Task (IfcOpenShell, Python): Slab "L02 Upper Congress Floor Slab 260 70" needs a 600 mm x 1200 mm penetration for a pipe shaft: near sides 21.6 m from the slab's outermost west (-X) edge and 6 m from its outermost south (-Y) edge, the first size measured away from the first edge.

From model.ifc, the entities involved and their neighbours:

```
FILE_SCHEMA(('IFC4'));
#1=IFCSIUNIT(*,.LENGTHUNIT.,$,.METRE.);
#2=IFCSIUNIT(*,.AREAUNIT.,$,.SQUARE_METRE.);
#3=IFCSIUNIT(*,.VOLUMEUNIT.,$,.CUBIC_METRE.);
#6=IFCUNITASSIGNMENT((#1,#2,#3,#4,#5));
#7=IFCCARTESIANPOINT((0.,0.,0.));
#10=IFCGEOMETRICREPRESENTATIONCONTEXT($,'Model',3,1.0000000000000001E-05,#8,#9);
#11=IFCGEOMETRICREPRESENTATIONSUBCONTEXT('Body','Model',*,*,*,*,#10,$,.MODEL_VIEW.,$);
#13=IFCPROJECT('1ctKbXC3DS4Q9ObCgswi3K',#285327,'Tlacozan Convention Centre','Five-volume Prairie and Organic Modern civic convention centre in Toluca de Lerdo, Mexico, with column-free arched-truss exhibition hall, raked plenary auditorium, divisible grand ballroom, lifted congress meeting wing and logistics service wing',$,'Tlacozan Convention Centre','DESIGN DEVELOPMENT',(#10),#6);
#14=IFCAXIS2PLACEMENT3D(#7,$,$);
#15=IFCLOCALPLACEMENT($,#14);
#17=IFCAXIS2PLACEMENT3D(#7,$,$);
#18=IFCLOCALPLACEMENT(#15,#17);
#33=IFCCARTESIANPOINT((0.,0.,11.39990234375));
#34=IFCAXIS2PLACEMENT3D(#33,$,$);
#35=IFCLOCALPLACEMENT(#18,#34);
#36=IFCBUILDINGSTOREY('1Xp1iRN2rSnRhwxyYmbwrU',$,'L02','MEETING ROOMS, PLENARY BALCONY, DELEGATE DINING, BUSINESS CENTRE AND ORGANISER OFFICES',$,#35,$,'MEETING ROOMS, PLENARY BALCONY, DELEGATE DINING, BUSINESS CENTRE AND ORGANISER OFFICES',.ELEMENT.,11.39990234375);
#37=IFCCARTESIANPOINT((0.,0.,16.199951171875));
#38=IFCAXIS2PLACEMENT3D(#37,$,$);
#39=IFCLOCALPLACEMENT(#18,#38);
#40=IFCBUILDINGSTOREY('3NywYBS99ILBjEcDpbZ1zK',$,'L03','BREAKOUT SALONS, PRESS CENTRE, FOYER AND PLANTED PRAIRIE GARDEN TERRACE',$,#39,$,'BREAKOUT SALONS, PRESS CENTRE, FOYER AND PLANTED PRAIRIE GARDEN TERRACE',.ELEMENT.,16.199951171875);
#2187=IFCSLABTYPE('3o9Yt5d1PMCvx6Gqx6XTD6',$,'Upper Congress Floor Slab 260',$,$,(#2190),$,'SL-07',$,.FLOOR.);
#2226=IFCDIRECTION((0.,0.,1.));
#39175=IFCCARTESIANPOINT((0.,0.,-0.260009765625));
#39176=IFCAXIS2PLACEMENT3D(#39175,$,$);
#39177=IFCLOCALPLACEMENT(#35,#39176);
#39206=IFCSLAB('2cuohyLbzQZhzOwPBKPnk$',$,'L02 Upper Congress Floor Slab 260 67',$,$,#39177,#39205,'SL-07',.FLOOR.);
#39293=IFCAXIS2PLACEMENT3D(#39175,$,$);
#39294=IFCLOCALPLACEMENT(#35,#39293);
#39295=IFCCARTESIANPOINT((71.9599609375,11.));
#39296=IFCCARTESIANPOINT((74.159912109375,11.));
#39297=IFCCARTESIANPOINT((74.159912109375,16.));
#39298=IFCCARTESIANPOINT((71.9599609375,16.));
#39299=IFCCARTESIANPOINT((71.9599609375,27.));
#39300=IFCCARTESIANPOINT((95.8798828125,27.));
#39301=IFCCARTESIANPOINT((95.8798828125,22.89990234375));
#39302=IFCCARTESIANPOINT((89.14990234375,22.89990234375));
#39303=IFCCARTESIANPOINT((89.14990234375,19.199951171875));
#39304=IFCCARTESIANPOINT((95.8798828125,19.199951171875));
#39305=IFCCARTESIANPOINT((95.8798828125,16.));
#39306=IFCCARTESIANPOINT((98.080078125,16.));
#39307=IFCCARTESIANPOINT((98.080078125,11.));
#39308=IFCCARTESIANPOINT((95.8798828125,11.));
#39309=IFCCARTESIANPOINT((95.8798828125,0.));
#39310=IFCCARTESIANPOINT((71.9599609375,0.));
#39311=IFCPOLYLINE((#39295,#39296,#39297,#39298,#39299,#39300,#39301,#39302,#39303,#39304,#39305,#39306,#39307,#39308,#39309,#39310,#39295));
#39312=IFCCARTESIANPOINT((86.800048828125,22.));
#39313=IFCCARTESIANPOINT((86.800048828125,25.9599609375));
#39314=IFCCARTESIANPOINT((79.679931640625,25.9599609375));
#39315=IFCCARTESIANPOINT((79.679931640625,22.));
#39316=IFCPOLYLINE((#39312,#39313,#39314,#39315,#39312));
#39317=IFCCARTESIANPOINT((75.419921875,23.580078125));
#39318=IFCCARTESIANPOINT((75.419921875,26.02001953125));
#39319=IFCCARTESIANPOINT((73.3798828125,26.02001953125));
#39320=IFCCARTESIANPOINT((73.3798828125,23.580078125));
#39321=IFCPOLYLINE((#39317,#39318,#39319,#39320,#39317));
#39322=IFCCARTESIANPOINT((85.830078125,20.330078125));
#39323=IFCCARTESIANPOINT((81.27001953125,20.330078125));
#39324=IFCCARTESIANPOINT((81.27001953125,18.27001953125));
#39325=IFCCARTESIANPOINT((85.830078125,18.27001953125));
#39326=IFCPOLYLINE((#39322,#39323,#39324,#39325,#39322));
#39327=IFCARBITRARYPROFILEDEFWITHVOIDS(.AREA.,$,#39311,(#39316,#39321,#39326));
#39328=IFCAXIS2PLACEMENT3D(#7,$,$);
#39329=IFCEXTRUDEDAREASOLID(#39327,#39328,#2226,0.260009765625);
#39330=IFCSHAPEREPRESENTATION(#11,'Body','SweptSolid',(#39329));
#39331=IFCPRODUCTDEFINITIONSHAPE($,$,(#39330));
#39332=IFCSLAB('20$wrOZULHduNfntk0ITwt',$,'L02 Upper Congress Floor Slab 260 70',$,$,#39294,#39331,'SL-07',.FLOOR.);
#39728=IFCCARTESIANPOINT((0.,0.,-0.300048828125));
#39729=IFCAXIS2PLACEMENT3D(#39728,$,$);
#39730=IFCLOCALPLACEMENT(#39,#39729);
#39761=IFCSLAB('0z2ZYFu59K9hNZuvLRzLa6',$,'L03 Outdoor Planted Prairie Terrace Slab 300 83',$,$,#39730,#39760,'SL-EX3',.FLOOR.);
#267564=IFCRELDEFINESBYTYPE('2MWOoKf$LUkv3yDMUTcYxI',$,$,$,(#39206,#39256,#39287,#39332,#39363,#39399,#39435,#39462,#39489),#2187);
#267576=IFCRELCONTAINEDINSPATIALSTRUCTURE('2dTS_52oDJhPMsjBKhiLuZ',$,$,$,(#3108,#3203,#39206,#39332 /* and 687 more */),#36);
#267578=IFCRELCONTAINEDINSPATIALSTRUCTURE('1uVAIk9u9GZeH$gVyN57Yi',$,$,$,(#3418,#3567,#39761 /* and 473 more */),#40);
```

```python
import numpy as np
import ifcopenshell
import ifcopenshell.api.feature
import ifcopenshell.api.geometry
import ifcopenshell.api.root
import ifcopenshell.geom
import ifcopenshell.util.placement
import ifcopenshell.util.representation
import ifcopenshell.util.shape
import ifcopenshell.util.unit

model = ifcopenshell.open("model.ifc")
unit_scale = ifcopenshell.util.unit.calculate_unit_scale(model)
settings = ifcopenshell.geom.settings()


def volume(element):
    """Net volume in cubic metres, openings subtracted."""
    shape = ifcopenshell.geom.create_shape(settings, element)
    return ifcopenshell.util.shape.get_volume(shape.geometry)


slab = model.by_id(39332)
before = volume(slab)

# Extent in the slab's own axes, in metres. The edges named are its -X and -Y sides.
slab_shape = ifcopenshell.geom.create_shape(settings, slab)
vertices = ifcopenshell.util.shape.get_vertices(slab_shape.geometry)
x_min, y_min, bottom = vertices.min(axis=0)
top = vertices[:, 2].max()

opening = ifcopenshell.api.root.create_entity(model, ifc_class="IfcOpeningElement", name="Pipe shaft opening", predefined_type="OPENING")
context = ifcopenshell.util.representation.get_context(model, "Model", "Body", "MODEL_VIEW")
width, depth = 0.6, 1.2
outline = [(0.0, 0.0), (width, 0.0), (width, depth), (0.0, depth), (0.0, 0.0)]
# Overshoot both faces by 50 mm so the cut is clean.
shape = ifcopenshell.api.geometry.add_slab_representation(
    model, context=context, depth=top - bottom + 0.1, polyline=outline
)
ifcopenshell.api.geometry.assign_representation(model, product=opening, representation=shape)

matrix = ifcopenshell.util.placement.get_local_placement(slab.ObjectPlacement)
matrix[:, 3] = matrix @ np.append(np.array([x_min + 21.6, y_min + 6, bottom - 0.05]) / unit_scale, 1.0)
ifcopenshell.api.geometry.edit_object_placement(model, product=opening, matrix=matrix, is_si=False)
ifcopenshell.api.feature.add_feature(model, feature=opening, element=slab)

after = volume(slab)

print(f"slab volume {before:.3f} -> {after:.3f} m3")

model.write("model-out.ifc")
```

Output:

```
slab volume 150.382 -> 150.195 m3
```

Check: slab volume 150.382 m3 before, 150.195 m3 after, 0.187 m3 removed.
